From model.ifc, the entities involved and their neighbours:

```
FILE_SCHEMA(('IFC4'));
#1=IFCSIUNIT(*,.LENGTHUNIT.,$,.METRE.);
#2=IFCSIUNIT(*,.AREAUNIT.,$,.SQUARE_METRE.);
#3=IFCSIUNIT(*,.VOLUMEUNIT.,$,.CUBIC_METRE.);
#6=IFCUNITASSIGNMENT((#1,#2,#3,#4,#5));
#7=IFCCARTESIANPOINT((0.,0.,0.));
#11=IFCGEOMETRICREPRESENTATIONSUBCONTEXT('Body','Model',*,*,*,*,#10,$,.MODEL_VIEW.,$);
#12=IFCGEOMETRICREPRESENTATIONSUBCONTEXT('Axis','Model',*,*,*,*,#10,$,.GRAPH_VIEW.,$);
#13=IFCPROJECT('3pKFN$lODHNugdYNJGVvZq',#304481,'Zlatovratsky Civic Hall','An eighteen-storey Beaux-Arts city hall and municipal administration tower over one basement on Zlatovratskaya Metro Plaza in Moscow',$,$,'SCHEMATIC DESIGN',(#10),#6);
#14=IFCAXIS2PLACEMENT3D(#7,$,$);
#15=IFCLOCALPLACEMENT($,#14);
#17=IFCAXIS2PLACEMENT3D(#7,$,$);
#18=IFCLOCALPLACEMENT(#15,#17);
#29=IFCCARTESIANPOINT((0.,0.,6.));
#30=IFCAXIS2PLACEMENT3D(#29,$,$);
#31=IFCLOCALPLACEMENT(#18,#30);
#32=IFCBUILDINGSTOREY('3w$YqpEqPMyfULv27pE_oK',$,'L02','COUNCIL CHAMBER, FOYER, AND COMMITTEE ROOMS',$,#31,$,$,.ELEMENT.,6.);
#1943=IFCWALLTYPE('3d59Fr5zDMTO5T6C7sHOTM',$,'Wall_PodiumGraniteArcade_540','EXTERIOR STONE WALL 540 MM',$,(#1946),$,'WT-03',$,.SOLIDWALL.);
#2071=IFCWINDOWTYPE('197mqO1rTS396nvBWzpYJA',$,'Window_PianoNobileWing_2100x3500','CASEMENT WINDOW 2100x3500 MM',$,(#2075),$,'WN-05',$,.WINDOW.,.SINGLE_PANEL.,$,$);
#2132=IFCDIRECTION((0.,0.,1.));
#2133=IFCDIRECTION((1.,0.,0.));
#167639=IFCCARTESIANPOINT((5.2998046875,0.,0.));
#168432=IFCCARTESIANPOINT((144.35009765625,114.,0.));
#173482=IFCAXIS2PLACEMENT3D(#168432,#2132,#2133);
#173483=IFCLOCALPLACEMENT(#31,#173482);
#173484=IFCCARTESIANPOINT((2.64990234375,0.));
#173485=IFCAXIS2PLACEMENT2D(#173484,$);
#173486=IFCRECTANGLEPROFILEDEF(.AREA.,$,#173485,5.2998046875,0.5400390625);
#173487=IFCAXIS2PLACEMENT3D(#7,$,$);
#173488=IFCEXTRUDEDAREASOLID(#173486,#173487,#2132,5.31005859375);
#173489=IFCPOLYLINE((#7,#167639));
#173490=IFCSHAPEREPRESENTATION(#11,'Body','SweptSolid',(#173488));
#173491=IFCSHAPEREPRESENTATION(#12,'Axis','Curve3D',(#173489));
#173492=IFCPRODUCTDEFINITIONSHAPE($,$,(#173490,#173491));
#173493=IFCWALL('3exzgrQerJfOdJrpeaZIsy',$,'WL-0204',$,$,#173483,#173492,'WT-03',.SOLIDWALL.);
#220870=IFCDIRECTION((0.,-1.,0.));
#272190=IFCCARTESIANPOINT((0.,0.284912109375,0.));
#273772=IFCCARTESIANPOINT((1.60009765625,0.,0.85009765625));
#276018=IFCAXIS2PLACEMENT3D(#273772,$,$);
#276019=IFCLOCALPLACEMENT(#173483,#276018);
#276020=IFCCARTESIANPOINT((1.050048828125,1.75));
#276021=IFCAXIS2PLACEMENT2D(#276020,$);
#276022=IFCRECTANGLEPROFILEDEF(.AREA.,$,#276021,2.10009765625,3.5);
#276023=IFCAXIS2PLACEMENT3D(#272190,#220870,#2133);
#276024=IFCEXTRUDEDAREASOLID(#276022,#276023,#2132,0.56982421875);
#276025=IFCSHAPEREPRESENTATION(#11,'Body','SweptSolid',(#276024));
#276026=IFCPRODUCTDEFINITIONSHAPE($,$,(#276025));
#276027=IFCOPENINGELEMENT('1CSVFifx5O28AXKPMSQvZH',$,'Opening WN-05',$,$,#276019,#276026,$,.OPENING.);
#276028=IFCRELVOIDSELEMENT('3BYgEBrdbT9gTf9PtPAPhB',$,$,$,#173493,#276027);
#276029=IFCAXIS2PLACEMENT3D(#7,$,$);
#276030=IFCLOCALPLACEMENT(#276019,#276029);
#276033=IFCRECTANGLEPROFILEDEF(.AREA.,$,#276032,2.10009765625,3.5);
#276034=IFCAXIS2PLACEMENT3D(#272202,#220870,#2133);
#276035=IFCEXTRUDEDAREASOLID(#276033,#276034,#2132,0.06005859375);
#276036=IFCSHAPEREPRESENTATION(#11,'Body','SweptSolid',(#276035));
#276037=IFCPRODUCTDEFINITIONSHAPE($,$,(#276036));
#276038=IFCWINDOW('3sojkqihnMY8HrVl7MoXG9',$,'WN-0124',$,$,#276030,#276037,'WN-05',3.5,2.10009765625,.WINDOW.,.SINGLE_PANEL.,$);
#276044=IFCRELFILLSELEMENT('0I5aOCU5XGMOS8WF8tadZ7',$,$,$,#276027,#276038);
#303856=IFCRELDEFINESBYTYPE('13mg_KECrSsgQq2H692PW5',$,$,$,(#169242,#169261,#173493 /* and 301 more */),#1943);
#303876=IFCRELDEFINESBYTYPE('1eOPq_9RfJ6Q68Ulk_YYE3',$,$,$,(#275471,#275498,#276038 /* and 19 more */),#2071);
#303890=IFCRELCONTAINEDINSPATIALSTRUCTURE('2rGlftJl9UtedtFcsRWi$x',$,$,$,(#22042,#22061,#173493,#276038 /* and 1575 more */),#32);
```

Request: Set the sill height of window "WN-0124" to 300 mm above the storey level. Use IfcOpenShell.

```python
import numpy as np
import ifcopenshell
import ifcopenshell.api.geometry
import ifcopenshell.geom
import ifcopenshell.util.element
import ifcopenshell.util.placement
import ifcopenshell.util.shape
import ifcopenshell.util.unit

model = ifcopenshell.open("model.ifc")
unit_scale = ifcopenshell.util.unit.calculate_unit_scale(model)

window = model.by_guid("3sojkqihnMY8HrVl7MoXG9")
opening = window.FillsVoids[0].RelatingOpeningElement
storey = ifcopenshell.util.element.get_container(window, ifc_class="IfcBuildingStorey")
level = ifcopenshell.util.placement.get_local_placement(storey.ObjectPlacement)[2, 3]

# The opening's origin need not be at the sill, so measure its lowest point.
shape = ifcopenshell.geom.create_shape(ifcopenshell.geom.settings(), opening)
bottom = ifcopenshell.util.shape.get_shape_bottom_elevation(shape, shape.geometry) / unit_scale
dz = level + 0.3 / unit_scale - bottom

shift = np.array([0.0, 0.0, dz])
# The window is placed relative to its opening, so it follows when the opening moves.
matrix = ifcopenshell.util.placement.get_local_placement(opening.ObjectPlacement)
matrix[:3, 3] += shift
ifcopenshell.api.geometry.edit_object_placement(
    model, product=opening, matrix=matrix, is_si=False, should_transform_children=True
)

print(f"moved by {dz * unit_scale:+.3f} m")

model.write("model-out.ifc")
```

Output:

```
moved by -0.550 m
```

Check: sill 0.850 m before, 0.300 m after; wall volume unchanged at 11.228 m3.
